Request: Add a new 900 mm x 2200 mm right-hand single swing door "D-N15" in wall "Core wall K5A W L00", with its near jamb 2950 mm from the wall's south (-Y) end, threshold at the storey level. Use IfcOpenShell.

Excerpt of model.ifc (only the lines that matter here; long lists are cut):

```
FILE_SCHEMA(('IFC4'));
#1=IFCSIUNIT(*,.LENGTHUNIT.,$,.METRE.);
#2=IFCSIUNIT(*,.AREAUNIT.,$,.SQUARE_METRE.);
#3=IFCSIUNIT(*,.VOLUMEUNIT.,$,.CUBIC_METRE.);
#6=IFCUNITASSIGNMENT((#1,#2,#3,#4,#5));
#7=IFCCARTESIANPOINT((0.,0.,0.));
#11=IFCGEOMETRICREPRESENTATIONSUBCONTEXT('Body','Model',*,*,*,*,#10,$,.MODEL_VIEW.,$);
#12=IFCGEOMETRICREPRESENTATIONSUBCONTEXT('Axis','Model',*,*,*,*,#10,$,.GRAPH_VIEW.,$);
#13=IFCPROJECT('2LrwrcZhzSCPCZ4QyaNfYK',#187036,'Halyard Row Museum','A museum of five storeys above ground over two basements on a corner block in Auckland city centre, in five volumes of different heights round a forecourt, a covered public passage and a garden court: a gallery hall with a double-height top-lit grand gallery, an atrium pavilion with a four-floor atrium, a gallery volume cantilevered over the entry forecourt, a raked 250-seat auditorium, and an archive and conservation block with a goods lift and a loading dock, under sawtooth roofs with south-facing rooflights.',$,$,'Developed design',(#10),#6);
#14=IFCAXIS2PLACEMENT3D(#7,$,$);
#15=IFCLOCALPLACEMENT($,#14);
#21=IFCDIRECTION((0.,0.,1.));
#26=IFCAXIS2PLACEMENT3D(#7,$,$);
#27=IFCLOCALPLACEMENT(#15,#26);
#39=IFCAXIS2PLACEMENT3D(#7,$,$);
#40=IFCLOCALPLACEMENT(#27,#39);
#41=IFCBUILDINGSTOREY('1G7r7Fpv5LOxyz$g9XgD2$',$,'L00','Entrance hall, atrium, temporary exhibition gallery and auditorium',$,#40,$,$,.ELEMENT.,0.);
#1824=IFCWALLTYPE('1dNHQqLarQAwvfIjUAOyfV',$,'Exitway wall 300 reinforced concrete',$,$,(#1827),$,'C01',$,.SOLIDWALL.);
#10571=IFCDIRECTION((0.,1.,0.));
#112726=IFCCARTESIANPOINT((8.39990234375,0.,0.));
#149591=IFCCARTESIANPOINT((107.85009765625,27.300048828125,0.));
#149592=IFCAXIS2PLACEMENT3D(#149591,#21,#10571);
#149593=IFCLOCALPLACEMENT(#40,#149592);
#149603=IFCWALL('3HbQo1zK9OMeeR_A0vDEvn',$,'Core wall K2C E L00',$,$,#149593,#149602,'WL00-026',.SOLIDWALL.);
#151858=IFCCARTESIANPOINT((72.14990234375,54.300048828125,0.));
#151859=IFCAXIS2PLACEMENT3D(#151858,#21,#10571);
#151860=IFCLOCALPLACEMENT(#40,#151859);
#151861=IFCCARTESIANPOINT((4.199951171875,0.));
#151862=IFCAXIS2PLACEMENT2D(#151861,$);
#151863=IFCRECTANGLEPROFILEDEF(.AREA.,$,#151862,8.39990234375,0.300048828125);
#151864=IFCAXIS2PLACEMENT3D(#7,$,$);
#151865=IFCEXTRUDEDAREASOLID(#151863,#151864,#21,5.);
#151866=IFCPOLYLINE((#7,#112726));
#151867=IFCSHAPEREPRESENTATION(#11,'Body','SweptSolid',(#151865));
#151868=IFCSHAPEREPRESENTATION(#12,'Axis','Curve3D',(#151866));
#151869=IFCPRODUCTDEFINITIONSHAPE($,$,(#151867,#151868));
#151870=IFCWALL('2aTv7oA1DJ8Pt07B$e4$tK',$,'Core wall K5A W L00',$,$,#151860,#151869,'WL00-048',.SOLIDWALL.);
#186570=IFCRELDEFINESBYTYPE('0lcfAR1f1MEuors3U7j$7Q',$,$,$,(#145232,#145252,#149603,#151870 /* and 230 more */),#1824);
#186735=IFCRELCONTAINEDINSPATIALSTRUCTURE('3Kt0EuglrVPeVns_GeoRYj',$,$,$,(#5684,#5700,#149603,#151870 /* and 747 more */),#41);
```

```python
import numpy as np
import ifcopenshell
import ifcopenshell.api.feature
import ifcopenshell.api.geometry
import ifcopenshell.api.root
import ifcopenshell.api.spatial
import ifcopenshell.geom
import ifcopenshell.util.element
import ifcopenshell.util.placement
import ifcopenshell.util.representation
import ifcopenshell.util.shape
import ifcopenshell.util.unit

model = ifcopenshell.open("model.ifc")
unit_scale = ifcopenshell.util.unit.calculate_unit_scale(model)
settings = ifcopenshell.geom.settings()


def volume(element):
    """Net volume in cubic metres, openings subtracted."""
    shape = ifcopenshell.geom.create_shape(settings, element)
    return ifcopenshell.util.shape.get_volume(shape.geometry)


wall = model.by_guid("2aTv7oA1DJ8Pt07B$e4$tK")
storey = ifcopenshell.util.element.get_container(wall, ifc_class="IfcBuildingStorey")
context = ifcopenshell.util.representation.get_context(model, "Model", "Body", "MODEL_VIEW")
before = volume(wall)

width, height, from_end, sill = 0.9, 2.2, 2.95, 0.0  # metres

# The wall runs along its own X axis, and the end named is its -X end.
wall_shape = ifcopenshell.geom.create_shape(settings, wall)
x, y, z = ifcopenshell.util.shape.get_vertices(wall_shape.geometry).T
start = x.min() + from_end
face, thickness = float(y.min()), float(y.max() - y.min())
wall_matrix = ifcopenshell.util.placement.get_local_placement(wall.ObjectPlacement)
level = ifcopenshell.util.placement.get_local_placement(storey.ObjectPlacement)[2, 3]


def in_wall(x, y):
    """Placement at x, y metres in the wall's axes, at sill height."""
    matrix = wall_matrix.copy()
    matrix[:, 3] = wall_matrix @ np.array([x / unit_scale, y / unit_scale, 0.0, 1.0])
    matrix[2, 3] = level + sill / unit_scale
    return matrix


# Opening: a box that overshoots both wall faces by 50 mm.
opening = ifcopenshell.api.root.create_entity(model, ifc_class="IfcOpeningElement", predefined_type="OPENING")
box = ifcopenshell.api.geometry.add_wall_representation(
    model, context=context, length=width, height=height, thickness=thickness + 0.1
)
ifcopenshell.api.geometry.assign_representation(model, product=opening, representation=box)
ifcopenshell.api.geometry.edit_object_placement(model, product=opening, matrix=in_wall(start, face - 0.05), is_si=False)
ifcopenshell.api.feature.add_feature(model, feature=opening, element=wall)

door = ifcopenshell.api.root.create_entity(model, ifc_class="IfcDoor", name="D-N15", predefined_type="DOOR")
door.OverallWidth, door.OverallHeight = width / unit_scale, height / unit_scale
door.OperationType = "SINGLE_SWING_RIGHT"
body = ifcopenshell.api.geometry.add_door_representation(
    model,
    context=context,
    overall_width=door.OverallWidth,
    overall_height=door.OverallHeight,
    operation_type="SINGLE_SWING_RIGHT",
    lining_properties={"LiningDepth": thickness / unit_scale, "ThresholdDepth": thickness / unit_scale},
)
ifcopenshell.api.geometry.assign_representation(model, product=door, representation=body)
ifcopenshell.api.spatial.assign_container(model, products=[door], relating_structure=storey)
ifcopenshell.api.feature.add_filling(model, opening=opening, element=door)

# The lining spans the wall, so the door starts at the wall face.
ifcopenshell.api.geometry.edit_object_placement(model, product=door, matrix=in_wall(start, face), is_si=False)

after = volume(wall)

print(f"wall volume {before:.3f} -> {after:.3f} m3")

model.write("model_edited.ifc")
```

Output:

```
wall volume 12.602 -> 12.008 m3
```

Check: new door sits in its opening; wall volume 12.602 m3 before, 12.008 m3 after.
